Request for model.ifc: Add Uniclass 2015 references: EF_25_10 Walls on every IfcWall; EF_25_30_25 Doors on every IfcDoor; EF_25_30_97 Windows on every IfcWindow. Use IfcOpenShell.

First a look at what the model holds.

```python
import ifcopenshell

model = ifcopenshell.open("model.ifc")
print(model.schema)
print("classifications:", [c.Name for c in model.by_type("IfcClassification")])
for ifc_class in ("IfcDoor", "IfcRoof", "IfcStair", "IfcWall", "IfcWindow"):
    print(ifc_class, len(model.by_type(ifc_class)))
```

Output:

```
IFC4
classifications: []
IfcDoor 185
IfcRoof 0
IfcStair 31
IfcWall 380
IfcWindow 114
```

```python
import ifcopenshell
import ifcopenshell.api.classification

model = ifcopenshell.open("model.ifc")

system = ifcopenshell.api.classification.add_classification(model, classification="Uniclass 2015")

codes = {
    "IfcWall": ("EF_25_10", "Walls"),
    "IfcDoor": ("EF_25_30_25", "Doors"),
    "IfcWindow": ("EF_25_30_97", "Windows"),
}
for ifc_class, (code, name) in codes.items():
    products = model.by_type(ifc_class)
    ifcopenshell.api.classification.add_reference(
        model, products=products, classification=system, identification=code, name=name
    )
    print(code, len(products))

model.write("model_v2.ifc")
```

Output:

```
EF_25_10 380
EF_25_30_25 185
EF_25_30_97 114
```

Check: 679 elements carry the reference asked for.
